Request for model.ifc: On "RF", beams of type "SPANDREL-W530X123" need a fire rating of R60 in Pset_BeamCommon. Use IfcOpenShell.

First a look at what the model holds.

```python
import ifcopenshell
import ifcopenshell.util.element

model = ifcopenshell.open("model.ifc")
print(model.schema)
storey = next(s for s in model.by_type("IfcBuildingStorey") if s.Name == "RF")
beams = [e for e in ifcopenshell.util.element.get_decomposition(storey) if e.is_a("IfcBeam")]
seen = {}
for e in beams:
    element_type = ifcopenshell.util.element.get_type(e)
    key = (element_type.Name if element_type != e and element_type else None, ifcopenshell.util.element.get_pset(e, "Pset_BeamCommon", "FireRating"))
    seen[key] = seen.get(key, 0) + 1
for (name, value), count in sorted(seen.items(), key=str):
    print(count, "x", name, "|", value)
```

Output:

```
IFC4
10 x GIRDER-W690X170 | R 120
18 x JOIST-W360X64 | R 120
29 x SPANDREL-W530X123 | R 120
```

```python
import ifcopenshell
import ifcopenshell.api.pset
import ifcopenshell.util.element

model = ifcopenshell.open("model.ifc")

storey = next(s for s in model.by_type("IfcBuildingStorey") if s.Name == "RF")
beams = [e for e in ifcopenshell.util.element.get_decomposition(storey) if e.is_a("IfcBeam")]

count = 0
for e in beams:
    element_type = ifcopenshell.util.element.get_type(e)
    if element_type in (None, e) or element_type.Name != "SPANDREL-W530X123":
        continue
    # add_pset returns the element's existing set when there is one.
    pset = ifcopenshell.api.pset.add_pset(model, product=e, name="Pset_BeamCommon")
    ifcopenshell.api.pset.edit_pset(model, pset=pset, properties={"FireRating": "R60"})
    count += 1

print(count, "beams updated")

model.write("model_v2.ifc")
```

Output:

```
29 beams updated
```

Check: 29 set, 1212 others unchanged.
